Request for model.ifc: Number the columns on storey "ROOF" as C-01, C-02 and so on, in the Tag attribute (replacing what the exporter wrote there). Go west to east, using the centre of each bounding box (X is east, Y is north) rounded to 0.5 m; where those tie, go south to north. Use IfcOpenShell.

First a look at what the model holds.

```python
import ifcopenshell
import ifcopenshell.util.element
import ifcopenshell.util.placement

model = ifcopenshell.open("model.ifc")
print(model.schema)
storey = next(s for s in model.by_type("IfcBuildingStorey") if s.Name == "ROOF")
columns = [e for e in ifcopenshell.util.element.get_decomposition(storey) if e.is_a("IfcColumn")]
for e in sorted(columns, key=lambda e: e.id()):
    origin = ifcopenshell.util.placement.get_local_placement(e.ObjectPlacement)[:3, 3]
    print(e.id(), e.Tag, e.Name, origin.round(2) + 0.0, sep=" | ")
```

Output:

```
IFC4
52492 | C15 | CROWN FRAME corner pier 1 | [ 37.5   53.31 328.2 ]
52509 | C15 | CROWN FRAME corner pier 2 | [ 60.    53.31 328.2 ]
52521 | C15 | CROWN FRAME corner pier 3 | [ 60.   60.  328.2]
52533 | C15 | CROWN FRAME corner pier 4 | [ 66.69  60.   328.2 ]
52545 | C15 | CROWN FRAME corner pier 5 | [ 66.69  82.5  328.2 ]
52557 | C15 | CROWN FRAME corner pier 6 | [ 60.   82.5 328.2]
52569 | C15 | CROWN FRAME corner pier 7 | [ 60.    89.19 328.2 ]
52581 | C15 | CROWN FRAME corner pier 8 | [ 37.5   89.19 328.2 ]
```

```python
import ifcopenshell
import ifcopenshell.geom
import ifcopenshell.util.element
import ifcopenshell.util.shape

model = ifcopenshell.open("model.ifc")
settings = ifcopenshell.geom.settings()
settings.set("use-world-coords", True)


def centre(element):
    shape = ifcopenshell.geom.create_shape(settings, element)
    return ifcopenshell.util.shape.get_bbox_centroid(shape.geometry)


storey = next(s for s in model.by_type("IfcBuildingStorey") if s.Name == "ROOF")
columns = [e for e in ifcopenshell.util.element.get_decomposition(storey) if e.is_a("IfcColumn")]

# Insertion points can sit at a corner or the storey origin, so sort by the geometry (in metres).
centres = {e: centre(e) for e in columns}
columns.sort(key=lambda e: (round(centres[e][0] / 0.5), centres[e][1]))

for i, e in enumerate(columns, start=1):
    number = f"C-{i:02d}"
    e.Tag = number
    print(e.id(), number)

model.write("model-out.ifc")
```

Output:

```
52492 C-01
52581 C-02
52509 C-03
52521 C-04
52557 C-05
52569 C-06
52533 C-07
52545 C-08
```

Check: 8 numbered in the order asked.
